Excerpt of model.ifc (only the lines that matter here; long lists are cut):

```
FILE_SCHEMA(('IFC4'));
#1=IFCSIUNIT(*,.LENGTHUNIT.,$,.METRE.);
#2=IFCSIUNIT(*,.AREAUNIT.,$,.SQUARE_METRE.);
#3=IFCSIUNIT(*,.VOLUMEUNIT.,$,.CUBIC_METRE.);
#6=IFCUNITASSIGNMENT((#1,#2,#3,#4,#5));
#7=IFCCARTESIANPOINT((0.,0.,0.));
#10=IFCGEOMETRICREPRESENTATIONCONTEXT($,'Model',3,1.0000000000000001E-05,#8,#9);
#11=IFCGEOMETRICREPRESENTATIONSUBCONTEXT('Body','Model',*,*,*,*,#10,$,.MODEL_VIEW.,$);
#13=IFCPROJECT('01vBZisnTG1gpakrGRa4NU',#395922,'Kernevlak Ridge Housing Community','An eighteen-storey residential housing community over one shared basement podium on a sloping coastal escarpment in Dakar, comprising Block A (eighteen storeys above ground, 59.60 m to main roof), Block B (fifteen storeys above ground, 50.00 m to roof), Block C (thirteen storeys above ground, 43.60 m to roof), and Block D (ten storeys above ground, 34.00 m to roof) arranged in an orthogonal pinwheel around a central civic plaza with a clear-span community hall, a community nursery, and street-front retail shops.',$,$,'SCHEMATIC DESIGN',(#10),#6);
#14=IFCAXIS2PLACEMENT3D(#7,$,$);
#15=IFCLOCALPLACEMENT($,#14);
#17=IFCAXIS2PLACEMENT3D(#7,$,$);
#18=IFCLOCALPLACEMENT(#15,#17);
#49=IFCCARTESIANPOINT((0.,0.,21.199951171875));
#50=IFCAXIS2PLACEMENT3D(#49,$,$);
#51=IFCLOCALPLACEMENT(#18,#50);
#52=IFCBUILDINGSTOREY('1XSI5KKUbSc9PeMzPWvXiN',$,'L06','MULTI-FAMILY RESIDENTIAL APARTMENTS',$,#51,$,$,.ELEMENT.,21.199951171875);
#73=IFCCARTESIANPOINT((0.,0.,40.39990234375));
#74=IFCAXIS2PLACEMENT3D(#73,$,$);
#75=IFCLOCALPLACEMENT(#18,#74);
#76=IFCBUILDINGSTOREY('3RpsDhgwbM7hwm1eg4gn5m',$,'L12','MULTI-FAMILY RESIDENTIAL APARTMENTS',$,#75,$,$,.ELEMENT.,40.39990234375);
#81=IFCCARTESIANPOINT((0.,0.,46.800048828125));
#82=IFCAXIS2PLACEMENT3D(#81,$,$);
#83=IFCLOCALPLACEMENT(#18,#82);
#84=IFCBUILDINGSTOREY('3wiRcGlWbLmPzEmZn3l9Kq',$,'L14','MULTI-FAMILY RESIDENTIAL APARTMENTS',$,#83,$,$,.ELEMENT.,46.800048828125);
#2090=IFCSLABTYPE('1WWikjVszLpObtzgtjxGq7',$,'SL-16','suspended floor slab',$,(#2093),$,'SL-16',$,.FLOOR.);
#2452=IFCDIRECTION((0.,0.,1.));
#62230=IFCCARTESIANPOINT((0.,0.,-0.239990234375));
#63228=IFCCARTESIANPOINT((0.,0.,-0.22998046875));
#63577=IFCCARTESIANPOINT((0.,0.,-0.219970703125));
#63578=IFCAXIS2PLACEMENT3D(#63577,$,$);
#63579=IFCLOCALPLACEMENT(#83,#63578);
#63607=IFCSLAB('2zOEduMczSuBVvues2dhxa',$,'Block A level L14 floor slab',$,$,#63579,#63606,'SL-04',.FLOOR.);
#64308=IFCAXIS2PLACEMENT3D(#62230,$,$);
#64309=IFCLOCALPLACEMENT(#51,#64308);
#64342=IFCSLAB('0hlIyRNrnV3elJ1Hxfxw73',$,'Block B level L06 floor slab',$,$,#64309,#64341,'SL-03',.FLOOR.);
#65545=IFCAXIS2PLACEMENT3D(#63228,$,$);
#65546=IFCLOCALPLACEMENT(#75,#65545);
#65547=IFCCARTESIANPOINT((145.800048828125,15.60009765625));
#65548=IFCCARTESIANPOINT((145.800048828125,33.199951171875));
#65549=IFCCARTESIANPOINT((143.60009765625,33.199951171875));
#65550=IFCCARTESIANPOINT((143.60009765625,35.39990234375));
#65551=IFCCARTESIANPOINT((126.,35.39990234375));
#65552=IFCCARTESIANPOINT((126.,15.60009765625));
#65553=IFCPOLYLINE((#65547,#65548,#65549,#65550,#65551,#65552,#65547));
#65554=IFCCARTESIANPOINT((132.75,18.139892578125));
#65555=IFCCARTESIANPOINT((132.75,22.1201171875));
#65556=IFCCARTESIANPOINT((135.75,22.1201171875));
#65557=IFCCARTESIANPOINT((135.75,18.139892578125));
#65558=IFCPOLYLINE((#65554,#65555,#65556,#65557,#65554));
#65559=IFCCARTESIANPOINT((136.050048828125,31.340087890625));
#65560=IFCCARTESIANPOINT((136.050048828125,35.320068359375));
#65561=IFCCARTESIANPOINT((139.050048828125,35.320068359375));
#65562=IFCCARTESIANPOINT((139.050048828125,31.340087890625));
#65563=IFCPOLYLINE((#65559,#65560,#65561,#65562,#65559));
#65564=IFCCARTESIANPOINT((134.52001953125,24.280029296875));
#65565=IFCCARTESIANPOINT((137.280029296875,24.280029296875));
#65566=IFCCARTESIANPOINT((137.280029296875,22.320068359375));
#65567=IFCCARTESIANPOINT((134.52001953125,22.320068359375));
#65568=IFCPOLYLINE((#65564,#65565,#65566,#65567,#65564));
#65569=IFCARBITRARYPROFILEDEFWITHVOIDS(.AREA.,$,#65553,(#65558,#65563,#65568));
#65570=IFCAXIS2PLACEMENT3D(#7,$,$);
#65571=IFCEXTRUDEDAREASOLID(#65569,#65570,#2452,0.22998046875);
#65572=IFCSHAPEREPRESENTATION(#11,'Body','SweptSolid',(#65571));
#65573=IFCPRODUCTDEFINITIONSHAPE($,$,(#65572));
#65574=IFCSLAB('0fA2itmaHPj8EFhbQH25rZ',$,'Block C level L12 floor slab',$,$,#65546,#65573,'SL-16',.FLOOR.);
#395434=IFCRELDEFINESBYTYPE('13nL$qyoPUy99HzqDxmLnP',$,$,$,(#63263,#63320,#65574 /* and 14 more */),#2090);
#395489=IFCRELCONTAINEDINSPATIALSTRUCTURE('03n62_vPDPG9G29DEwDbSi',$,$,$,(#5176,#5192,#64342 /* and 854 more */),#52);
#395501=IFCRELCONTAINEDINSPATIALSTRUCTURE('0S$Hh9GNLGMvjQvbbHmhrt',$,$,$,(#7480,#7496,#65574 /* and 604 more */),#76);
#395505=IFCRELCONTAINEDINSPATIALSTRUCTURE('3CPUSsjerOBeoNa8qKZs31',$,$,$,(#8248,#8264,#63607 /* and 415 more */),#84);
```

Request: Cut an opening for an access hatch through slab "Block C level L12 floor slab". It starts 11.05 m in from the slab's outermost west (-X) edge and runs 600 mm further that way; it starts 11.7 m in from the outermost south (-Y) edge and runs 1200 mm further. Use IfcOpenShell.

```python
import numpy as np
import ifcopenshell
import ifcopenshell.api.feature
import ifcopenshell.api.geometry
import ifcopenshell.api.root
import ifcopenshell.geom
import ifcopenshell.util.placement
import ifcopenshell.util.representation
import ifcopenshell.util.shape
import ifcopenshell.util.unit

model = ifcopenshell.open("model.ifc")
unit_scale = ifcopenshell.util.unit.calculate_unit_scale(model)
settings = ifcopenshell.geom.settings()


def volume(element):
    """Net volume in cubic metres, openings subtracted."""
    shape = ifcopenshell.geom.create_shape(settings, element)
    return ifcopenshell.util.shape.get_volume(shape.geometry)


slab = model.by_guid("0fA2itmaHPj8EFhbQH25rZ")
before = volume(slab)

# Extent in the slab's own axes, in metres. The edges named are its -X and -Y sides.
slab_shape = ifcopenshell.geom.create_shape(settings, slab)
vertices = ifcopenshell.util.shape.get_vertices(slab_shape.geometry)
x_min, y_min, bottom = vertices.min(axis=0)
top = vertices[:, 2].max()

opening = ifcopenshell.api.root.create_entity(model, ifc_class="IfcOpeningElement", name="Access hatch opening", predefined_type="OPENING")
context = ifcopenshell.util.representation.get_context(model, "Model", "Body", "MODEL_VIEW")
width, depth = 0.6, 1.2
outline = [(0.0, 0.0), (width, 0.0), (width, depth), (0.0, depth), (0.0, 0.0)]
# Overshoot both faces by 50 mm so the cut is clean.
shape = ifcopenshell.api.geometry.add_slab_representation(
    model, context=context, depth=top - bottom + 0.1, polyline=outline
)
ifcopenshell.api.geometry.assign_representation(model, product=opening, representation=shape)

matrix = ifcopenshell.util.placement.get_local_placement(slab.ObjectPlacement)
matrix[:, 3] = matrix @ np.append(np.array([x_min + 11.05, y_min + 11.7, bottom - 0.05]) / unit_scale, 1.0)
ifcopenshell.api.geometry.edit_object_placement(model, product=opening, matrix=matrix, is_si=False)
ifcopenshell.api.feature.add_feature(model, feature=opening, element=slab)

after = volume(slab)

print(f"slab volume {before:.3f} -> {after:.3f} m3")

model.write("model_edited.ifc")
```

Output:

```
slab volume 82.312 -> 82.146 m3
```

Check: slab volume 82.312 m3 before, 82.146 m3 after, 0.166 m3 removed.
